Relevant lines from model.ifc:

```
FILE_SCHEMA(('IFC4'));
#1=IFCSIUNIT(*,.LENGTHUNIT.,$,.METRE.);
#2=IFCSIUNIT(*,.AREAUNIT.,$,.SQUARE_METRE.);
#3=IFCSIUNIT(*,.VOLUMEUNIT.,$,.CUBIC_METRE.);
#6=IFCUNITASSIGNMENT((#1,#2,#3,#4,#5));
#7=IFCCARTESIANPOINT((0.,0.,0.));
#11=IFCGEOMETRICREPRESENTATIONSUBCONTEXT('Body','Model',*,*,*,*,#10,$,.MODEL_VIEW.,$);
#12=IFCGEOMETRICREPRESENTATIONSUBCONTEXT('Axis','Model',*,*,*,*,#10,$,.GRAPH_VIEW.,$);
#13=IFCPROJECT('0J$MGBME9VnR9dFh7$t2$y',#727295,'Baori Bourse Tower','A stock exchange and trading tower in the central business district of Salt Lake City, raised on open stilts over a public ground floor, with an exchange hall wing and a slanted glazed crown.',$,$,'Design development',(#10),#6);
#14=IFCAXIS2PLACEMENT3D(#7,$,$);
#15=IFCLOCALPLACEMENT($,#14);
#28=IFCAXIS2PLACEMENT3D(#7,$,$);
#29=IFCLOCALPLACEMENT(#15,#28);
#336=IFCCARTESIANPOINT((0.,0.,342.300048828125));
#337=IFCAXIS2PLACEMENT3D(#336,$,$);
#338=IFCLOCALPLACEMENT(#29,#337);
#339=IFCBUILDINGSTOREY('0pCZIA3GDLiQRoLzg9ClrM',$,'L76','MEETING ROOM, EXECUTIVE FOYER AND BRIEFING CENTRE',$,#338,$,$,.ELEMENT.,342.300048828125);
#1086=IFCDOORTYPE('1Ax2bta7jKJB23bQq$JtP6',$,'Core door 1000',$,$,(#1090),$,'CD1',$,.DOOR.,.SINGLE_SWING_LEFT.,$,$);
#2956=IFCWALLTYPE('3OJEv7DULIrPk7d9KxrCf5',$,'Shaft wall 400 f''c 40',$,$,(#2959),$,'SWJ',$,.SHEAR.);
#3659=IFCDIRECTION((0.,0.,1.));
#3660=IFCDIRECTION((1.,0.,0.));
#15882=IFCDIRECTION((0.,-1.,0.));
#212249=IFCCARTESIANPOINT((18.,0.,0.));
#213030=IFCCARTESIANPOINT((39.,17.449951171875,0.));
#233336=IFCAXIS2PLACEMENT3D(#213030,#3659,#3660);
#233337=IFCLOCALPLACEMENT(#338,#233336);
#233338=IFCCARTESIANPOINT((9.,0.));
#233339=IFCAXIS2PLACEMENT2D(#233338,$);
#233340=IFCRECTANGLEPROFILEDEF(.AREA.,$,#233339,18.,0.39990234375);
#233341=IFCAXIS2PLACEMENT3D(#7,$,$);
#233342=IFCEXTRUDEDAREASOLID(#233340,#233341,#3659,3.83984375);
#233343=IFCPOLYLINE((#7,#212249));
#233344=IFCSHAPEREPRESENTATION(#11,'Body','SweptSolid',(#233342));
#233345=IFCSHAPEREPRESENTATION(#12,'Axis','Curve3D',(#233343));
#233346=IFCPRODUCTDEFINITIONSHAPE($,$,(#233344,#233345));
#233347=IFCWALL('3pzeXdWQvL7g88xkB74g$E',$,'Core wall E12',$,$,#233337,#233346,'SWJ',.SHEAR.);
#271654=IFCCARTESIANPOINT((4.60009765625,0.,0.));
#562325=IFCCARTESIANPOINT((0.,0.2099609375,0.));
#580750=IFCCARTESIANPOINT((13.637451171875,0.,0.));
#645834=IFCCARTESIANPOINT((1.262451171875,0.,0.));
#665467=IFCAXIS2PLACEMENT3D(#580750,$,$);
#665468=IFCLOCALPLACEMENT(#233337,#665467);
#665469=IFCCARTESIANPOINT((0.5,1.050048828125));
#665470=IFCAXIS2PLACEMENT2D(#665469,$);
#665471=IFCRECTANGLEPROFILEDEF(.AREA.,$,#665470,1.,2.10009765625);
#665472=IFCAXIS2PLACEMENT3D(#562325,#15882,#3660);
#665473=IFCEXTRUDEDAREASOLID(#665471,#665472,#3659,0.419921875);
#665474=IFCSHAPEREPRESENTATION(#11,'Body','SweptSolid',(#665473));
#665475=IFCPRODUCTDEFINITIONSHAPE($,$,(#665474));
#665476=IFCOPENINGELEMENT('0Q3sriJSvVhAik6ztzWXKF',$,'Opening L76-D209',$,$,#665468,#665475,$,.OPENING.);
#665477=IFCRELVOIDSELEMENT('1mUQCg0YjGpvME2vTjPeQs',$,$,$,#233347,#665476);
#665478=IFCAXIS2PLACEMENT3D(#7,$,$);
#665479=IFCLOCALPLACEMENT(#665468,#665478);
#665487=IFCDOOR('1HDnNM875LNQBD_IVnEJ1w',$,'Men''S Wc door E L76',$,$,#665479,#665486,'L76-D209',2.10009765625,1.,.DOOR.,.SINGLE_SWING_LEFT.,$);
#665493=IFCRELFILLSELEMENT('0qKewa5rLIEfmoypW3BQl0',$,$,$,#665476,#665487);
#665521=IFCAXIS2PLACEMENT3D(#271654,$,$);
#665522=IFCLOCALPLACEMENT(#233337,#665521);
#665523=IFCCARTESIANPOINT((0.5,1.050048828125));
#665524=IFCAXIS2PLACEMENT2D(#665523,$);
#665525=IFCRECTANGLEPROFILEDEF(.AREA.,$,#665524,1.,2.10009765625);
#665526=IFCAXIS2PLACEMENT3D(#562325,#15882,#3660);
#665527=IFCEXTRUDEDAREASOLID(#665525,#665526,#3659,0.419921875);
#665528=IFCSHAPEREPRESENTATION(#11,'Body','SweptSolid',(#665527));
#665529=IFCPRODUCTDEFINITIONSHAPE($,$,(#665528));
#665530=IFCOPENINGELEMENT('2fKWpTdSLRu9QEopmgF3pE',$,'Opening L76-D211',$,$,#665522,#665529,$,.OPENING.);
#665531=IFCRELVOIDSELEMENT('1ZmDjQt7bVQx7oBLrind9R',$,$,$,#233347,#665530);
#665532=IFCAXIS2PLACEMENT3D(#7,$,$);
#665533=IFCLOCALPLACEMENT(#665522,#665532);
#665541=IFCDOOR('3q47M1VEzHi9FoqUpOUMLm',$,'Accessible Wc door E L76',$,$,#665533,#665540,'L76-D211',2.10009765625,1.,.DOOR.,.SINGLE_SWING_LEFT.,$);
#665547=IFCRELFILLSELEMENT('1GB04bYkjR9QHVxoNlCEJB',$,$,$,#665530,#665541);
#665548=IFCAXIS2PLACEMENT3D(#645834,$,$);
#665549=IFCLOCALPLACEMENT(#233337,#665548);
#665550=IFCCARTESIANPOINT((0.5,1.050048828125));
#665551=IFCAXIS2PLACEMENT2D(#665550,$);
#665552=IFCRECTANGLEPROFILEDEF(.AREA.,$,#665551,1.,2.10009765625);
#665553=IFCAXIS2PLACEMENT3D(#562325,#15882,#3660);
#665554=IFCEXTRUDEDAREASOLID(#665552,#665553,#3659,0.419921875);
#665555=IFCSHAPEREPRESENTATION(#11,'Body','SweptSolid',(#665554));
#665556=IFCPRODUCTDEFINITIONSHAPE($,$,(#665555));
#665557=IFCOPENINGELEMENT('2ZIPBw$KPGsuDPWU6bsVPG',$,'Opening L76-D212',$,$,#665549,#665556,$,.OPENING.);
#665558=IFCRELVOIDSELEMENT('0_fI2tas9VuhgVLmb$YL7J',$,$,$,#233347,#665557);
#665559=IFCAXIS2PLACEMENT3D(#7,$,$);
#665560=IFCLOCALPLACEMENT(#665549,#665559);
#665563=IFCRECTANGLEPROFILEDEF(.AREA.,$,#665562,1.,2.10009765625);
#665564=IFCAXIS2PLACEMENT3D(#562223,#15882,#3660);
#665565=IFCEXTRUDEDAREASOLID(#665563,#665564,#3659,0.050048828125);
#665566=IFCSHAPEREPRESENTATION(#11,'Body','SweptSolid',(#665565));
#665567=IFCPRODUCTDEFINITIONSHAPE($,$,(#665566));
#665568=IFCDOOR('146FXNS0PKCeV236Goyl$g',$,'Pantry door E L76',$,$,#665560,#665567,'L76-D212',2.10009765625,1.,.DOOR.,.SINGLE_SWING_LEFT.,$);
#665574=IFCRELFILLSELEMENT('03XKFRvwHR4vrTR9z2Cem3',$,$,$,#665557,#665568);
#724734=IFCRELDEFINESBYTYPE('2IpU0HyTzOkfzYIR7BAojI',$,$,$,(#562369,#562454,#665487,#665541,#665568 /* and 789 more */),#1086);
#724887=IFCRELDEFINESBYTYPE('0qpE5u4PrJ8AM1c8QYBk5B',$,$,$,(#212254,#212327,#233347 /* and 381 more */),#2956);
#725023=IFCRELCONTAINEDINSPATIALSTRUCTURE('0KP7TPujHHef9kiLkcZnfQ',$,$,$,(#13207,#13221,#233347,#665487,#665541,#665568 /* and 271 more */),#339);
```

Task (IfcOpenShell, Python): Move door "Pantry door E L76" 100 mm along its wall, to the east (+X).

```python
import ifcopenshell
import ifcopenshell.api.geometry
import ifcopenshell.util.placement
import ifcopenshell.util.unit

model = ifcopenshell.open("model.ifc")
unit_scale = ifcopenshell.util.unit.calculate_unit_scale(model)

door = model.by_guid("146FXNS0PKCeV236Goyl$g")
opening = door.FillsVoids[0].RelatingOpeningElement
wall = opening.VoidsElements[0].RelatingBuildingElement

wall_matrix = ifcopenshell.util.placement.get_local_placement(wall.ObjectPlacement)
shift = wall_matrix[:3, 0] * 0.1 / unit_scale
before = ifcopenshell.util.placement.get_local_placement(door.ObjectPlacement)[:3, 3].copy()

# The door is placed relative to its opening, so it follows when the opening moves.
matrix = ifcopenshell.util.placement.get_local_placement(opening.ObjectPlacement)
matrix[:3, 3] += shift
ifcopenshell.api.geometry.edit_object_placement(
    model, product=opening, matrix=matrix, is_si=False, should_transform_children=True
)

after = ifcopenshell.util.placement.get_local_placement(door.ObjectPlacement)[:3, 3]
print("door moved by", (after - before).round(3) + 0.0)

model.write("model_updated.ifc")
```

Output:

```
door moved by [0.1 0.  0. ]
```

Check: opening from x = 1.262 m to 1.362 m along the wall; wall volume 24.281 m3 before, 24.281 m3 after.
